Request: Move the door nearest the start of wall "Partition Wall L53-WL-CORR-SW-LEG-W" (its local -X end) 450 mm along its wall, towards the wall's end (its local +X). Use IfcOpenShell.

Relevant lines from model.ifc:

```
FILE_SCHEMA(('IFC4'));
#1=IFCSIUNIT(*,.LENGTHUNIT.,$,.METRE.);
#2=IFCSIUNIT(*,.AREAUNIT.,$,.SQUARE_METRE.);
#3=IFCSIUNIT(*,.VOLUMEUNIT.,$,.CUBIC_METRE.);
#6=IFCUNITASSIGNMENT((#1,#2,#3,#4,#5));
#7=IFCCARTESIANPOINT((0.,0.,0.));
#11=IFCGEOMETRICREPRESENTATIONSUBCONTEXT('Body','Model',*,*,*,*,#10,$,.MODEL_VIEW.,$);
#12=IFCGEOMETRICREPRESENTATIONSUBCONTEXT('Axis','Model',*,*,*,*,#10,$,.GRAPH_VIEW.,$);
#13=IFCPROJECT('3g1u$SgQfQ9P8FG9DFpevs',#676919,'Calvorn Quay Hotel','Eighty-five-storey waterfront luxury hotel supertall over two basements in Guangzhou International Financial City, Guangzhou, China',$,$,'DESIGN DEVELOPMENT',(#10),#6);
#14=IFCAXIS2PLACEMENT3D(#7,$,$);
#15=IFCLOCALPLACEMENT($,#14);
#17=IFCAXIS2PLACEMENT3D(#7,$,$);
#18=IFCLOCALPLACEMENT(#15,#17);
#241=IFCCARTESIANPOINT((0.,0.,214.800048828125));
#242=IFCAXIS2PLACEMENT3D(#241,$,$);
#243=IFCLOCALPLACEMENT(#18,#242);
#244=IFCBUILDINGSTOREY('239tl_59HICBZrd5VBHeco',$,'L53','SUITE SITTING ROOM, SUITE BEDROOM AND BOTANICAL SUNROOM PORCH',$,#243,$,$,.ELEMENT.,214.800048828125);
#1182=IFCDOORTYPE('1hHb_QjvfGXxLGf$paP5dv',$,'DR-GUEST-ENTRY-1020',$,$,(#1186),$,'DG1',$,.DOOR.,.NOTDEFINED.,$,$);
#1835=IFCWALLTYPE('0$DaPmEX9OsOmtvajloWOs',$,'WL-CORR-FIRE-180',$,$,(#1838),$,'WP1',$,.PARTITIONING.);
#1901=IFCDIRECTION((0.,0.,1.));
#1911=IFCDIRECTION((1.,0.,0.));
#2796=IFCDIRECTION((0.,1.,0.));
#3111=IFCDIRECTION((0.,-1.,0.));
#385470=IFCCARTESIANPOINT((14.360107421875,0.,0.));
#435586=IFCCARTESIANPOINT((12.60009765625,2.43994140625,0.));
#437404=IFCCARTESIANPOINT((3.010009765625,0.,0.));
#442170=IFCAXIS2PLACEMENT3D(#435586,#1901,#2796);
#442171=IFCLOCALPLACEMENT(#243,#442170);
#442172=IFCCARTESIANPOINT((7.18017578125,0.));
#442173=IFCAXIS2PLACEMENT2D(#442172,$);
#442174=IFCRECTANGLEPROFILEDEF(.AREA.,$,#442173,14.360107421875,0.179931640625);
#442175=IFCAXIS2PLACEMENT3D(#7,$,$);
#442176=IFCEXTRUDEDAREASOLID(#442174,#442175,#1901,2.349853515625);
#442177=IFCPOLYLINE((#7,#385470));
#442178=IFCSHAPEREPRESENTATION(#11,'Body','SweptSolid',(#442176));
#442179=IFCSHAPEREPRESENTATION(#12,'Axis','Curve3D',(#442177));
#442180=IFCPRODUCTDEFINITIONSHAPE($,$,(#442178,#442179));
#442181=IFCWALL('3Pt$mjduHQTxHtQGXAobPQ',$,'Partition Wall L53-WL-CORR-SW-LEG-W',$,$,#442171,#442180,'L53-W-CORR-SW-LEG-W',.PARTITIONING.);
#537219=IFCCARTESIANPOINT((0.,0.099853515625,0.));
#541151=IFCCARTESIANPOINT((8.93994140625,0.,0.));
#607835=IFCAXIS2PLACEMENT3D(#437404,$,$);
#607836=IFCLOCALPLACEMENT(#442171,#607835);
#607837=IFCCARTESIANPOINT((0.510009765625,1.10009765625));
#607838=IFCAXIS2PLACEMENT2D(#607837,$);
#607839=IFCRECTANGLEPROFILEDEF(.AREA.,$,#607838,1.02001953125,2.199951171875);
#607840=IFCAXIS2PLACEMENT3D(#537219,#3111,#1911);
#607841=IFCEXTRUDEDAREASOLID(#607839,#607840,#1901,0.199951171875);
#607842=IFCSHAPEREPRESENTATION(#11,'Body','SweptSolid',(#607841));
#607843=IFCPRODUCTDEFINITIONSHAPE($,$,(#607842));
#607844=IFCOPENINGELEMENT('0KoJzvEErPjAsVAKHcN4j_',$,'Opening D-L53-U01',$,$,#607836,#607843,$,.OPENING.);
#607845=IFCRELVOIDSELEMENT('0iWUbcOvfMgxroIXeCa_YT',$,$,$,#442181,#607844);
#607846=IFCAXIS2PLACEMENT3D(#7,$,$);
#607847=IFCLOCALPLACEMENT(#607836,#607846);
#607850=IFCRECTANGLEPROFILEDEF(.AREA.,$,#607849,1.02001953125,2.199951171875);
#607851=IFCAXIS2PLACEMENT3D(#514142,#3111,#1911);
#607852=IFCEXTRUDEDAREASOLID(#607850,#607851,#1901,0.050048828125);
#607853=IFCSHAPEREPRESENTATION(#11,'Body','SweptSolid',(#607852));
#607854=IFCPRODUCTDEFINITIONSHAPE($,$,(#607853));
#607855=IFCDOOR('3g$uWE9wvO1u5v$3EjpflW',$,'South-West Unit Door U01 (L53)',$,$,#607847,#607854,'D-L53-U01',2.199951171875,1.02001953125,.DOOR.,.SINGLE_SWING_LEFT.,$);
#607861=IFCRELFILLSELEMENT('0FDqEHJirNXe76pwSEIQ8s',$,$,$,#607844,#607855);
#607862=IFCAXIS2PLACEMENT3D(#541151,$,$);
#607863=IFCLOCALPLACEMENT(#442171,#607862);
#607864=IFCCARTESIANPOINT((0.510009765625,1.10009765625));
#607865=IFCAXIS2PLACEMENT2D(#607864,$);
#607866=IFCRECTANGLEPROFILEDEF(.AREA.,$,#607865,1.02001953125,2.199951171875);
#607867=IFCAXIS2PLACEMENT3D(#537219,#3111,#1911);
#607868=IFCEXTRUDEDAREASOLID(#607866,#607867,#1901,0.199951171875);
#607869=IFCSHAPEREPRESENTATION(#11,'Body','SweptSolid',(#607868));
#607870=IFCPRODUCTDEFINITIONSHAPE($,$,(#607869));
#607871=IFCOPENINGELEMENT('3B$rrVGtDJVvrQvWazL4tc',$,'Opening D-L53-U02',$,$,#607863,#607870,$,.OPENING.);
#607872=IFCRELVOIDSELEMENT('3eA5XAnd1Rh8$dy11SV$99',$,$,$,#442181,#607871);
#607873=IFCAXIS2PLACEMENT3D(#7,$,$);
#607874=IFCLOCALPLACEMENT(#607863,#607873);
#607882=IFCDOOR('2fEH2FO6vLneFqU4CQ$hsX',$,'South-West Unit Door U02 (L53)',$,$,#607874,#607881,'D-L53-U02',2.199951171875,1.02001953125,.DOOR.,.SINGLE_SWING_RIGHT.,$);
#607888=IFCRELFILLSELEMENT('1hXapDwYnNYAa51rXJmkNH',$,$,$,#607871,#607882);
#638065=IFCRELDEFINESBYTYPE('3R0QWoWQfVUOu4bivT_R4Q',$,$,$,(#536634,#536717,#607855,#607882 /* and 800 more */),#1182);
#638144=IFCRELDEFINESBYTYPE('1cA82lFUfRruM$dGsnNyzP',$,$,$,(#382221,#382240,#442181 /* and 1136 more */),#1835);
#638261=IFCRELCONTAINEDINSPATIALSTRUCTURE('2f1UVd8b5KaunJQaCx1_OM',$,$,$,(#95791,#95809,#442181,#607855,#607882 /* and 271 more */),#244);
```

```python
import ifcopenshell
import ifcopenshell.api.geometry
import ifcopenshell.util.placement
import ifcopenshell.util.unit

model = ifcopenshell.open("model.ifc")
unit_scale = ifcopenshell.util.unit.calculate_unit_scale(model)

door = model.by_guid("3g$uWE9wvO1u5v$3EjpflW")
opening = door.FillsVoids[0].RelatingOpeningElement
wall = opening.VoidsElements[0].RelatingBuildingElement

wall_matrix = ifcopenshell.util.placement.get_local_placement(wall.ObjectPlacement)
shift = wall_matrix[:3, 0] * 0.45 / unit_scale
before = ifcopenshell.util.placement.get_local_placement(door.ObjectPlacement)[:3, 3].copy()

# The door is placed relative to its opening, so it follows when the opening moves.
matrix = ifcopenshell.util.placement.get_local_placement(opening.ObjectPlacement)
matrix[:3, 3] += shift
ifcopenshell.api.geometry.edit_object_placement(
    model, product=opening, matrix=matrix, is_si=False, should_transform_children=True
)

after = ifcopenshell.util.placement.get_local_placement(door.ObjectPlacement)[:3, 3]
print("door moved by", (after - before).round(3) + 0.0)

model.write("model-out.ifc")
```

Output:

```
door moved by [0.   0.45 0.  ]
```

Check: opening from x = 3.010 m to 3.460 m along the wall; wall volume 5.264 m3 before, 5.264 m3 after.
